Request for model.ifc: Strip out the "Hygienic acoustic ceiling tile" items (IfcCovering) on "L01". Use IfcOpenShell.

First a look at what the model holds.

```python
import ifcopenshell
import ifcopenshell.util.element

model = ifcopenshell.open("model.ifc")
print(model.schema)
storey = next(s for s in model.by_type("IfcBuildingStorey") if s.Name == "L01")
coverings = [e for e in ifcopenshell.util.element.get_decomposition(storey) if e.is_a("IfcCovering")]
seen = {}
for e in coverings:
    element_type = ifcopenshell.util.element.get_type(e)
    name = element_type.Name if element_type not in (None, e) else None
    seen[name] = seen.get(name, 0) + 1
for name, count in sorted(seen.items(), key=str):
    print(count, "x", name)
```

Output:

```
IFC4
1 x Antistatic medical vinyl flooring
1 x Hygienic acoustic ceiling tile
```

```python
import ifcopenshell
import ifcopenshell.api.root
import ifcopenshell.util.element

model = ifcopenshell.open("model.ifc")

storey = next(s for s in model.by_type("IfcBuildingStorey") if s.Name == "L01")
coverings = [e for e in ifcopenshell.util.element.get_decomposition(storey) if e.is_a("IfcCovering")]
targets = [e for e in coverings if (t := ifcopenshell.util.element.get_type(e)) not in (None, e) and t.Name == "Hygienic acoustic ceiling tile"]

for e in targets:
    ifcopenshell.api.root.remove_product(model, product=e)
print(len(targets), "removed")

model.write("model_v2.ifc")
```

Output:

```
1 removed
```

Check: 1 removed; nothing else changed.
